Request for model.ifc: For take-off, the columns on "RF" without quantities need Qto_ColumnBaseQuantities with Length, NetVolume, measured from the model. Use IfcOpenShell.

First a look at what the model holds.

```python
import ifcopenshell
import ifcopenshell.util.element
import ifcopenshell.util.unit

model = ifcopenshell.open("model.ifc")
print(model.schema)
for unit_type in ("LENGTHUNIT", "AREAUNIT", "VOLUMEUNIT"):
    print(unit_type, ifcopenshell.util.unit.calculate_unit_scale(model, unit_type))
storey = next(s for s in model.by_type("IfcBuildingStorey") if s.Name == "RF")
columns = [e for e in ifcopenshell.util.element.get_decomposition(storey) if e.is_a("IfcColumn")]
for e in sorted(columns, key=lambda e: e.id()):
    print(e.id(), e.is_a(), e.Name, list(ifcopenshell.util.element.get_psets(e, qtos_only=True)), sep=" | ")
```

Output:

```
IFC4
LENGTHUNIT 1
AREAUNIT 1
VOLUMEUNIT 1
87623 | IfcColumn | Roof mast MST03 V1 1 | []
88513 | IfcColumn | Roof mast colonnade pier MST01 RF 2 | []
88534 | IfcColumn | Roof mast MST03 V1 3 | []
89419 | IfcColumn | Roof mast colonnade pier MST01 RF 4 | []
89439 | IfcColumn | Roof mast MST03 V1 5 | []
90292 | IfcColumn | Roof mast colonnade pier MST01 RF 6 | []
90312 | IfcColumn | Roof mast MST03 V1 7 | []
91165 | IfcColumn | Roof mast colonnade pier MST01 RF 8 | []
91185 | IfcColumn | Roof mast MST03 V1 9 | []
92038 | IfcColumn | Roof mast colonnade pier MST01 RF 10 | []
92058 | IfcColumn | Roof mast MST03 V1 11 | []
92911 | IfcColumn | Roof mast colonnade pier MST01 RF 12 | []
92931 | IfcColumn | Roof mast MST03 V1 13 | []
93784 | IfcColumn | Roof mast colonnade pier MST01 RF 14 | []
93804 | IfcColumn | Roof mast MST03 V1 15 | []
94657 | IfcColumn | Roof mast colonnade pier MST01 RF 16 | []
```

```python
import ifcopenshell
import ifcopenshell.api.pset
import ifcopenshell.geom
import ifcopenshell.util.element
import ifcopenshell.util.shape
import ifcopenshell.util.unit

model = ifcopenshell.open("model.ifc")
unit_scale = ifcopenshell.util.unit.calculate_unit_scale(model)
volume_scale = ifcopenshell.util.unit.calculate_unit_scale(model, "VOLUMEUNIT")
settings = ifcopenshell.geom.settings()

storey = next(s for s in model.by_type("IfcBuildingStorey") if s.Name == "RF")
columns = [e for e in ifcopenshell.util.element.get_decomposition(storey) if e.is_a("IfcColumn")]

for e in sorted(columns, key=lambda e: e.id()):
    if ifcopenshell.util.element.get_psets(e, qtos_only=True, should_inherit=False):
        continue
    # Geometry comes back in metres, in the element's own axes.
    shape = ifcopenshell.geom.create_shape(settings, e)
    values = {
        "Length": ifcopenshell.util.shape.get_z(shape.geometry) / unit_scale,
        "NetVolume": ifcopenshell.util.shape.get_volume(shape.geometry) / volume_scale,
    }
    qto = ifcopenshell.api.pset.add_qto(model, product=e, name="Qto_ColumnBaseQuantities")
    ifcopenshell.api.pset.edit_qto(model, qto=qto, properties=values)
    print(e.id(), {k: round(v, 3) for k, v in values.items()})

model.write("model_updated.ifc")
```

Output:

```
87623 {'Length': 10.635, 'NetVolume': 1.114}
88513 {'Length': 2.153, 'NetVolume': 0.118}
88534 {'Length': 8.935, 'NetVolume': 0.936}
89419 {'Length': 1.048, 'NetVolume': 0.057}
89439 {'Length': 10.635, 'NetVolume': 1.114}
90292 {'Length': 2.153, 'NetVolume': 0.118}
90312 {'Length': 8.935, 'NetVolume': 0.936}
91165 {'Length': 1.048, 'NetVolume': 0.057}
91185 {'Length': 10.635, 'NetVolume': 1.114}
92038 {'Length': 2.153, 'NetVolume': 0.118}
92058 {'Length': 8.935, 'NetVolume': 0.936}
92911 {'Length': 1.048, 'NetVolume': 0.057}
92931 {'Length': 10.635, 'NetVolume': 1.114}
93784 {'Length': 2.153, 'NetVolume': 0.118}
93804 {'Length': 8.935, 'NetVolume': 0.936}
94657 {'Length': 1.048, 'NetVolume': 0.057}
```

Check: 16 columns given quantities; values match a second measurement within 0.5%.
